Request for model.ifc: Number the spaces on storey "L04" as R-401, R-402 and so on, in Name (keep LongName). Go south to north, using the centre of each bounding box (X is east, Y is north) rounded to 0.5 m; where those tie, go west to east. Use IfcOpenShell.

First a look at what the model holds.

```python
import ifcopenshell
import ifcopenshell.util.element
import ifcopenshell.util.placement

model = ifcopenshell.open("model.ifc")
print(model.schema)
storey = next(s for s in model.by_type("IfcBuildingStorey") if s.Name == "L04")
spaces = [e for e in ifcopenshell.util.element.get_decomposition(storey) if e.is_a("IfcSpace")]
for e in sorted(spaces, key=lambda e: e.id()):
    origin = ifcopenshell.util.placement.get_local_placement(e.ObjectPlacement)[:3, 3]
    print(e.id(), e.Name, e.LongName, origin.round(2) + 0.0, sep=" | ")
```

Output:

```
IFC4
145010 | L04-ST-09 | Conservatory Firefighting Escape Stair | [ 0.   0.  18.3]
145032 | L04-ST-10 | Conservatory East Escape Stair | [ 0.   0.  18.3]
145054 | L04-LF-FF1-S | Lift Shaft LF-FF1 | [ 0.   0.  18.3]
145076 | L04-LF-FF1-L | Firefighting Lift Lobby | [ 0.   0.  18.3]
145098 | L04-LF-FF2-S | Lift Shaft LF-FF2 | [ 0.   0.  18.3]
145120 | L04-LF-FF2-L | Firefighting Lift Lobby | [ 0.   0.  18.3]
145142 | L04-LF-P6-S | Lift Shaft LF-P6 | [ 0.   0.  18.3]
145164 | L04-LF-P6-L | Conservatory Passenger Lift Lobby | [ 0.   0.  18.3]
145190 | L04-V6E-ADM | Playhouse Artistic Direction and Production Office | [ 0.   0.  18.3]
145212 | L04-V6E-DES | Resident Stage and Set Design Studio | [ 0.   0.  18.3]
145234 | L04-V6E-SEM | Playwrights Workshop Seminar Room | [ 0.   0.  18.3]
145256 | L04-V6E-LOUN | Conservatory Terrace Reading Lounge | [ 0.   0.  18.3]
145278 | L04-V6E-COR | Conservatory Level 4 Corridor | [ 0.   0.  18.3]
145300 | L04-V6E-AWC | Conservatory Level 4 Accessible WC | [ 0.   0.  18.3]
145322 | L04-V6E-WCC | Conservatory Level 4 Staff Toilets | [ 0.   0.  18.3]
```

```python
import ifcopenshell
import ifcopenshell.geom
import ifcopenshell.util.element
import ifcopenshell.util.shape

model = ifcopenshell.open("model.ifc")
settings = ifcopenshell.geom.settings()
settings.set("use-world-coords", True)


def centre(element):
    shape = ifcopenshell.geom.create_shape(settings, element)
    return ifcopenshell.util.shape.get_bbox_centroid(shape.geometry)


storey = next(s for s in model.by_type("IfcBuildingStorey") if s.Name == "L04")
spaces = [e for e in ifcopenshell.util.element.get_decomposition(storey) if e.is_a("IfcSpace")]

# Insertion points can sit at a corner or the storey origin, so sort by the geometry (in metres).
centres = {e: centre(e) for e in spaces}
spaces.sort(key=lambda e: (round(centres[e][1] / 0.5), centres[e][0]))

for i, e in enumerate(spaces, start=1):
    number = f"R-4{i:02d}"
    e.Name = number
    print(e.id(), number)

model.write("model_rev.ifc")
```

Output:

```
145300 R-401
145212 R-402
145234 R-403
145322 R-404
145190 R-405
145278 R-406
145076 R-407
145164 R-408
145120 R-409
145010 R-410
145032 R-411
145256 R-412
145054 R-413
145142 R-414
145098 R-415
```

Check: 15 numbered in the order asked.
